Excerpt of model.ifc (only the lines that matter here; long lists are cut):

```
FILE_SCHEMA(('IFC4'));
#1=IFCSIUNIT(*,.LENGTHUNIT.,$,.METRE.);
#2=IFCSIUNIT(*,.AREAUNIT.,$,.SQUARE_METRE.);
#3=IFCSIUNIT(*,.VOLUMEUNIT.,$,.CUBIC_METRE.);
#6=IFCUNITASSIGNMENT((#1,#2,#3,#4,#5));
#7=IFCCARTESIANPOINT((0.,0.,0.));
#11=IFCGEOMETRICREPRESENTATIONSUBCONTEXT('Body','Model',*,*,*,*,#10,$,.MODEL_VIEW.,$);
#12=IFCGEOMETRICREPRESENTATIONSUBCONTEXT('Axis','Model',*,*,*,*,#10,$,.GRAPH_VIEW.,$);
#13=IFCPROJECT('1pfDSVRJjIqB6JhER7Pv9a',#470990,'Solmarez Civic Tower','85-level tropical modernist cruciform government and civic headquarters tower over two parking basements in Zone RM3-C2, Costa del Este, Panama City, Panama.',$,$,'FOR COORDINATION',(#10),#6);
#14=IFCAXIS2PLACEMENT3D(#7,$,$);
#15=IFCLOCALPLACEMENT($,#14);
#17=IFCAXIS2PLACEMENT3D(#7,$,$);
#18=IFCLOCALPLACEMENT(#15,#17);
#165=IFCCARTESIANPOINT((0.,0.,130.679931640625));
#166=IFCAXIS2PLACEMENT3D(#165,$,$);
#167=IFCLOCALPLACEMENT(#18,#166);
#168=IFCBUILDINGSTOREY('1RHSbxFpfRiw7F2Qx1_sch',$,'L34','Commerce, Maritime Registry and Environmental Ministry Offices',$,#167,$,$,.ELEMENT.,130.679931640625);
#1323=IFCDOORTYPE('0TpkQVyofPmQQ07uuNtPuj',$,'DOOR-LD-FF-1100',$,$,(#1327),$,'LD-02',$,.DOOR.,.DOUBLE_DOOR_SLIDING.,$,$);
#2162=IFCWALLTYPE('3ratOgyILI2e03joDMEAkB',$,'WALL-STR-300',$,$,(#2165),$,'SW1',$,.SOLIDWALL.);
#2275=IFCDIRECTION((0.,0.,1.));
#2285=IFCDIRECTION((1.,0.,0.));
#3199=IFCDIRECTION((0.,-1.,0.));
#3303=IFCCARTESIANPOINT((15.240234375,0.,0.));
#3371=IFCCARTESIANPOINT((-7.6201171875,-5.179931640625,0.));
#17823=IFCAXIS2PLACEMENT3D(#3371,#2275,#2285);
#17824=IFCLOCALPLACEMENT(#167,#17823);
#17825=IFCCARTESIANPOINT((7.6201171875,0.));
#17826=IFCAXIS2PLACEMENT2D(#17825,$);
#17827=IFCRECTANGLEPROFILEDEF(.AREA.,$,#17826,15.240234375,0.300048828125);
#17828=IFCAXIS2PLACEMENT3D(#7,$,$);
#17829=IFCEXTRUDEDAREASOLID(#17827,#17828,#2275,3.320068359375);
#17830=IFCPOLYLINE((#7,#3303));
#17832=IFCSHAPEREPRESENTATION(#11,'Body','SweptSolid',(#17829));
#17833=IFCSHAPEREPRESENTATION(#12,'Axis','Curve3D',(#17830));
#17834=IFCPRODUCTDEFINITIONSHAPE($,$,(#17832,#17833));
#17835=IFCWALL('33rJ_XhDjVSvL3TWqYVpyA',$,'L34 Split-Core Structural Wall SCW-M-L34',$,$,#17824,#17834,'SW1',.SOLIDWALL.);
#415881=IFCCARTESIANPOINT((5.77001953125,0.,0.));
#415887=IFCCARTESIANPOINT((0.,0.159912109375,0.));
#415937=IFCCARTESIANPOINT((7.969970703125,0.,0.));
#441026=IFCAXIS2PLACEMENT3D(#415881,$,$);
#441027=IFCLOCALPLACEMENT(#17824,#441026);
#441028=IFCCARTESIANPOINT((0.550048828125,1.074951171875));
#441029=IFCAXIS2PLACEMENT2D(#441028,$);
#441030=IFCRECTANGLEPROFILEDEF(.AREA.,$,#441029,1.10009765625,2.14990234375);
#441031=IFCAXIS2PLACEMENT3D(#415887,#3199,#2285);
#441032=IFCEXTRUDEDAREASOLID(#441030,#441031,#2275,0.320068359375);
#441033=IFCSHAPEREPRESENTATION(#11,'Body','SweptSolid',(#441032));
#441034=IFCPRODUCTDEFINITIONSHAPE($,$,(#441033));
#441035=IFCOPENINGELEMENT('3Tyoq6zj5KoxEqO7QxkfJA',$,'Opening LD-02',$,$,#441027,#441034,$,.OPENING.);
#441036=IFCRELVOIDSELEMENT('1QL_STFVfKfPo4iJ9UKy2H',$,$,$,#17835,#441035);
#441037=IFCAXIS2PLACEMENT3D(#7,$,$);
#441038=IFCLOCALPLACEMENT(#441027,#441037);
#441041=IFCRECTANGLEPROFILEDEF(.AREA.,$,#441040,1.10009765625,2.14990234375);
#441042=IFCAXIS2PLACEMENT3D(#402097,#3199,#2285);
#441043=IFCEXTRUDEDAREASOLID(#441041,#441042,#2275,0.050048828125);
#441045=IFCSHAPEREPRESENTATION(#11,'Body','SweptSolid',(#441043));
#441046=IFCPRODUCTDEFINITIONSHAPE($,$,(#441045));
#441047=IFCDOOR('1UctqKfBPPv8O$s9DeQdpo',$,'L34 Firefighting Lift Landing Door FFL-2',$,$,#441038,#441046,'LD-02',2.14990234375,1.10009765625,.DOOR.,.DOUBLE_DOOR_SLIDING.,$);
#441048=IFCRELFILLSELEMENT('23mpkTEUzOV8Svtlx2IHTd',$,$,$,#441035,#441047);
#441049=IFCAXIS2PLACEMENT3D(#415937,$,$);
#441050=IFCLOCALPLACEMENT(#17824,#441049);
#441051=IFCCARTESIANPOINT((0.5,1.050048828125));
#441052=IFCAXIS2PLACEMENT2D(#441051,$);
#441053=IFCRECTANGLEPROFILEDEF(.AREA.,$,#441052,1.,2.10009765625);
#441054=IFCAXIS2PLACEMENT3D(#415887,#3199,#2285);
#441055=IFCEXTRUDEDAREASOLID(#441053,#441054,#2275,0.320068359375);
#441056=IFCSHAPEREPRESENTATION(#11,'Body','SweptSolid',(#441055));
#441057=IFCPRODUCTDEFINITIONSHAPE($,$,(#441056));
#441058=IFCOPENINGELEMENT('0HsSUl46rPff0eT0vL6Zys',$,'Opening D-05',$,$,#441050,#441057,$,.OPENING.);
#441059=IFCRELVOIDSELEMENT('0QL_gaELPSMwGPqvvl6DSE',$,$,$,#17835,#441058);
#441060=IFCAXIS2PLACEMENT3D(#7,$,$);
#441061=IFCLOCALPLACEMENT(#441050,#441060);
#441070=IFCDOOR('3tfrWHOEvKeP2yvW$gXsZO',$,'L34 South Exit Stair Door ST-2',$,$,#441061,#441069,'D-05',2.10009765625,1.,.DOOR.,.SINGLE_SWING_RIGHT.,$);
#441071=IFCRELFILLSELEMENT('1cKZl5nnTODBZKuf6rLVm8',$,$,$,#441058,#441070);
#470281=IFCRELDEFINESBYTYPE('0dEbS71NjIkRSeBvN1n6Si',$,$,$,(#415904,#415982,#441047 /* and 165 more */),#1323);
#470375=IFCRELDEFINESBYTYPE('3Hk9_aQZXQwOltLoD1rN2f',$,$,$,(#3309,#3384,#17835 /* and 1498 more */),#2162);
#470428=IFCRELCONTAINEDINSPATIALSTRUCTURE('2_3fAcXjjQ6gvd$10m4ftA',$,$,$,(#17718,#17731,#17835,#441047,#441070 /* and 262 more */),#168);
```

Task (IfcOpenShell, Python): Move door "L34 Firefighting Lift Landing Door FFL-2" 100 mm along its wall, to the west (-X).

```python
import ifcopenshell
import ifcopenshell.api.geometry
import ifcopenshell.util.placement

model = ifcopenshell.open("model.ifc")

door = model.by_guid("1UctqKfBPPv8O$s9DeQdpo")
opening = door.FillsVoids[0].RelatingOpeningElement
wall = opening.VoidsElements[0].RelatingBuildingElement

wall_matrix = ifcopenshell.util.placement.get_local_placement(wall.ObjectPlacement)
shift = wall_matrix[:3, 0] * -0.1
before = ifcopenshell.util.placement.get_local_placement(door.ObjectPlacement)[:3, 3].copy()

# The door is placed relative to its opening, so it follows when the opening moves.
matrix = ifcopenshell.util.placement.get_local_placement(opening.ObjectPlacement)
matrix[:3, 3] += shift
ifcopenshell.api.geometry.edit_object_placement(
    model, product=opening, matrix=matrix, is_si=False, should_transform_children=True
)

after = ifcopenshell.util.placement.get_local_placement(door.ObjectPlacement)[:3, 3]
print("door moved by", (after - before).round(3) + 0.0)

model.write("model_edited.ifc")
```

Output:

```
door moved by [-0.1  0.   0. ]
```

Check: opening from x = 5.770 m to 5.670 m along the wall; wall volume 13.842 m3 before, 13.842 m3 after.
